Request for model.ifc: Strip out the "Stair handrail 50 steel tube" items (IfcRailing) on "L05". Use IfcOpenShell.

First a look at what the model holds.

```python
import ifcopenshell
import ifcopenshell.util.element

model = ifcopenshell.open("model.ifc")
print(model.schema)
storey = next(s for s in model.by_type("IfcBuildingStorey") if s.Name == "L05")
railings = [e for e in ifcopenshell.util.element.get_decomposition(storey) if e.is_a("IfcRailing")]
seen = {}
for e in railings:
    element_type = ifcopenshell.util.element.get_type(e)
    name = element_type.Name if element_type not in (None, e) else None
    seen[name] = seen.get(name, 0) + 1
for name, count in sorted(seen.items(), key=str):
    print(count, "x", name)
```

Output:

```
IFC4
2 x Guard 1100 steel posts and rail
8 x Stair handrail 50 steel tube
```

```python
import ifcopenshell
import ifcopenshell.api.root
import ifcopenshell.util.element

model = ifcopenshell.open("model.ifc")

storey = next(s for s in model.by_type("IfcBuildingStorey") if s.Name == "L05")
railings = [e for e in ifcopenshell.util.element.get_decomposition(storey) if e.is_a("IfcRailing")]
targets = [e for e in railings if (t := ifcopenshell.util.element.get_type(e)) not in (None, e) and t.Name == "Stair handrail 50 steel tube"]

for e in targets:
    ifcopenshell.api.root.remove_product(model, product=e)
print(len(targets), "removed")

model.write("model_rev.ifc")
```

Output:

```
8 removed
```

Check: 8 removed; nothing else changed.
